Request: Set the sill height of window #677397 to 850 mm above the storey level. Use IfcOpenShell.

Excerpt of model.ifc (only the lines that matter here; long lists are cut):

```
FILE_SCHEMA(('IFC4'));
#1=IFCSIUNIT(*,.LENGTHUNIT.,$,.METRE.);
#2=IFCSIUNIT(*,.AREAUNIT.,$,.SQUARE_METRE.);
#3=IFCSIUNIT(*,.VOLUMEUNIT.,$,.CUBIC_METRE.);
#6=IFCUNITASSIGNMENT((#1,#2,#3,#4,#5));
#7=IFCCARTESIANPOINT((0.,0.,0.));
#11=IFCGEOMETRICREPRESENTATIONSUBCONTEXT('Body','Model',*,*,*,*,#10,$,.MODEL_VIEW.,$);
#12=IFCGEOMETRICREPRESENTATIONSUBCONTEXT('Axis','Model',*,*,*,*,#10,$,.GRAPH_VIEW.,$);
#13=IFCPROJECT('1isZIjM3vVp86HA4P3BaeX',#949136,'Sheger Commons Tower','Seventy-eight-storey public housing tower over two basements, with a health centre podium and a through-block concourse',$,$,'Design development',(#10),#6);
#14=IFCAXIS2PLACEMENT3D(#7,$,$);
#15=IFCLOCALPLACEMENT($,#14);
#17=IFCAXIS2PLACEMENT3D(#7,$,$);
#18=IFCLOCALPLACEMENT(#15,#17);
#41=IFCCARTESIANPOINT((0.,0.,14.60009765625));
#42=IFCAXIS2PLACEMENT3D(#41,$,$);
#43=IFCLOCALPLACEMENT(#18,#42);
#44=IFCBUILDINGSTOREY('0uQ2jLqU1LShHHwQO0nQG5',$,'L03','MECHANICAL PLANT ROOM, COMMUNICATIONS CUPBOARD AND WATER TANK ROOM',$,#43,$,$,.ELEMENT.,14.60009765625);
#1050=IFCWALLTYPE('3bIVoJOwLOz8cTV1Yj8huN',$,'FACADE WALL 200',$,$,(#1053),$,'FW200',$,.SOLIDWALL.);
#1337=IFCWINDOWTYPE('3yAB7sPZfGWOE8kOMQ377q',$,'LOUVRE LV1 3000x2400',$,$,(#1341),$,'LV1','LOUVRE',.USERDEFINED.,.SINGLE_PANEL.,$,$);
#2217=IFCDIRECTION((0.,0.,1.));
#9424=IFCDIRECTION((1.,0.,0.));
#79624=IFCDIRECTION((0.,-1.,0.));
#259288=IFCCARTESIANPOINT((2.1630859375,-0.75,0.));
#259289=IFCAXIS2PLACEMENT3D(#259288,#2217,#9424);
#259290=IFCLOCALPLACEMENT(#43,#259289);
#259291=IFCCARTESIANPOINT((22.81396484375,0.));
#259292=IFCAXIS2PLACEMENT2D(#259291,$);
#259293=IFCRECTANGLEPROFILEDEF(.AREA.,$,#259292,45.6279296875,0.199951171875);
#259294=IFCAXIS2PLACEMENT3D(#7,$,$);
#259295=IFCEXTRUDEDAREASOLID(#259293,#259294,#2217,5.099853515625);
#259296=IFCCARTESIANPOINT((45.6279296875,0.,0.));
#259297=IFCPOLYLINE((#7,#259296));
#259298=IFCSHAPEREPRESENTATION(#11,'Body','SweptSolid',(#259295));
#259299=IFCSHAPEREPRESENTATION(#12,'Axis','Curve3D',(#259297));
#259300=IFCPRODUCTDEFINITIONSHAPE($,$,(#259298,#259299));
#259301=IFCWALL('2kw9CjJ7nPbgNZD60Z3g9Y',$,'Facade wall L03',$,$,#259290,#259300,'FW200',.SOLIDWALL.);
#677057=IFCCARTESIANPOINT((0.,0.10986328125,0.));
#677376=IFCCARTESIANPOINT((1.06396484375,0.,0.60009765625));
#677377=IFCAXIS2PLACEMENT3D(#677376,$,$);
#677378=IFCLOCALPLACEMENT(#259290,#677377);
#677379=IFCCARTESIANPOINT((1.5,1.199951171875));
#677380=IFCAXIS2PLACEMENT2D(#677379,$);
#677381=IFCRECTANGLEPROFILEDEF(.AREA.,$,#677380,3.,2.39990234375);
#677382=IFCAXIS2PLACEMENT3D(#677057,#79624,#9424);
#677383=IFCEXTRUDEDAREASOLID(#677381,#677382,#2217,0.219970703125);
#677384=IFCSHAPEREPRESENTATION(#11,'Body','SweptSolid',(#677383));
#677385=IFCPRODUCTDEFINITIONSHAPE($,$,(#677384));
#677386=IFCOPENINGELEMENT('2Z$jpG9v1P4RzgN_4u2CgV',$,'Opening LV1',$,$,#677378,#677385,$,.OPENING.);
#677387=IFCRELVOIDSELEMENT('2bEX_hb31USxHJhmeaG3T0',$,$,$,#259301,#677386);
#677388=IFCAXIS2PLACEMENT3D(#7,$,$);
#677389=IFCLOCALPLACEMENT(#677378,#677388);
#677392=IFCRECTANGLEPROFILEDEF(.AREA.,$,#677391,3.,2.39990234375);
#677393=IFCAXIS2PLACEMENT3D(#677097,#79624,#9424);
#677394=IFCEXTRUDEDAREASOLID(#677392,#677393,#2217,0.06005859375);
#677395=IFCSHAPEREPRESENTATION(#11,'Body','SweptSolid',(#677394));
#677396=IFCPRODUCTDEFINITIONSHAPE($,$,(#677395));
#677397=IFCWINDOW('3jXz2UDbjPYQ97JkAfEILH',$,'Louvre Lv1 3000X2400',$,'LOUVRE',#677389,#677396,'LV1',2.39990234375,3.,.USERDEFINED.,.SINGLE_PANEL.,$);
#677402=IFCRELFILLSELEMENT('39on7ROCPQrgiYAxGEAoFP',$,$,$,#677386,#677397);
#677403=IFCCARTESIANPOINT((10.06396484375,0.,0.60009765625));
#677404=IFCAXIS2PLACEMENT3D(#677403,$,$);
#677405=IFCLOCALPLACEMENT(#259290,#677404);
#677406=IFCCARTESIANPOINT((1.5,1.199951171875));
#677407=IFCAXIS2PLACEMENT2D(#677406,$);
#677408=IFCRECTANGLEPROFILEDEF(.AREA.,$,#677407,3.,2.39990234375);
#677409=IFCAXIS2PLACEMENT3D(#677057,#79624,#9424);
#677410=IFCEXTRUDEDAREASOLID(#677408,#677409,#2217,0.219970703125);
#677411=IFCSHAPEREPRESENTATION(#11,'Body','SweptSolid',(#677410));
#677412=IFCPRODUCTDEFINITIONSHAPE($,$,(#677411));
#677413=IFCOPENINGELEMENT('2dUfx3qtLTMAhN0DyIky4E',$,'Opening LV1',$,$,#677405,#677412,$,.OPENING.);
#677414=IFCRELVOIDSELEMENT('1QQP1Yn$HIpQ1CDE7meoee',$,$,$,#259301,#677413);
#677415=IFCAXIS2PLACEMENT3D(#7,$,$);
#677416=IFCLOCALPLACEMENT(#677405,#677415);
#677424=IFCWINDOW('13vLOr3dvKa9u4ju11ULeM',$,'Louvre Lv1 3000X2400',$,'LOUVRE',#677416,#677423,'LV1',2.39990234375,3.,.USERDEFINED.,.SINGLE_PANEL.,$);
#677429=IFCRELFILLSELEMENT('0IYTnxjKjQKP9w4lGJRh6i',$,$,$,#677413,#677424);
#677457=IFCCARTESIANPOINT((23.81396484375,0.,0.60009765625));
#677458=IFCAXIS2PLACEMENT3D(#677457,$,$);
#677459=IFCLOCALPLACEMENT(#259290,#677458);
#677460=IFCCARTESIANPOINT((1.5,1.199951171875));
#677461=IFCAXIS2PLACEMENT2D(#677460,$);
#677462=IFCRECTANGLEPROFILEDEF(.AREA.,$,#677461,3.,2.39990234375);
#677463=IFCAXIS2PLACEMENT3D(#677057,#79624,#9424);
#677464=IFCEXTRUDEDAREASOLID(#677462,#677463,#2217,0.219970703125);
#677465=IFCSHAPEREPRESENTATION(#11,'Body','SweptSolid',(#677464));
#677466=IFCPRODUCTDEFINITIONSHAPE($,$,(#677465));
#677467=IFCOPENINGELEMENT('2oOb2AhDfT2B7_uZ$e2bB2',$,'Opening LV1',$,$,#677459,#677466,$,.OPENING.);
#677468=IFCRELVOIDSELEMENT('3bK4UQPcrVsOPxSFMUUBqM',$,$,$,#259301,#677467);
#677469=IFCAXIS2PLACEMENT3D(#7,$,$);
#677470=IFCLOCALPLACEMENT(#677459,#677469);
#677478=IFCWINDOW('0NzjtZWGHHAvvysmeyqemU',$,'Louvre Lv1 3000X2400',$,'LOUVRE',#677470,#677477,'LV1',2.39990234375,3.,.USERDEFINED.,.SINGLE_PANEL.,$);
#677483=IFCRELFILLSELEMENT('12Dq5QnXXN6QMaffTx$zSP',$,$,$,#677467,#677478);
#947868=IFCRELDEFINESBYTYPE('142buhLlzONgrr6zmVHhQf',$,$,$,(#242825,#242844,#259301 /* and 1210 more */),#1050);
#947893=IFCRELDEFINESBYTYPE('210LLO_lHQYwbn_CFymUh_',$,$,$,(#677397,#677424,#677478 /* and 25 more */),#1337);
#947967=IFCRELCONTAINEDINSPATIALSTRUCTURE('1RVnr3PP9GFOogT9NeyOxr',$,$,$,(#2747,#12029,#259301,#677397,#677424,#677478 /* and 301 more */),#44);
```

```python
import numpy as np
import ifcopenshell
import ifcopenshell.api.geometry
import ifcopenshell.geom
import ifcopenshell.util.element
import ifcopenshell.util.placement
import ifcopenshell.util.shape
import ifcopenshell.util.unit

model = ifcopenshell.open("model.ifc")
unit_scale = ifcopenshell.util.unit.calculate_unit_scale(model)

window = model.by_id(677397)
opening = window.FillsVoids[0].RelatingOpeningElement
storey = ifcopenshell.util.element.get_container(window, ifc_class="IfcBuildingStorey")
level = ifcopenshell.util.placement.get_local_placement(storey.ObjectPlacement)[2, 3]

# The opening's origin need not be at the sill, so measure its lowest point.
shape = ifcopenshell.geom.create_shape(ifcopenshell.geom.settings(), opening)
bottom = ifcopenshell.util.shape.get_shape_bottom_elevation(shape, shape.geometry) / unit_scale
dz = level + 0.85 - bottom

shift = np.array([0.0, 0.0, dz])
# The window is placed relative to its opening, so it follows when the opening moves.
matrix = ifcopenshell.util.placement.get_local_placement(opening.ObjectPlacement)
matrix[:3, 3] += shift
ifcopenshell.api.geometry.edit_object_placement(
    model, product=opening, matrix=matrix, is_si=False, should_transform_children=True
)

print(f"moved by {dz * unit_scale:+.3f} m")

model.write("model_v2.ifc")
```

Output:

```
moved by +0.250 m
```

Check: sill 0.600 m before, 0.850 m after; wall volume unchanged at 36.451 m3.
